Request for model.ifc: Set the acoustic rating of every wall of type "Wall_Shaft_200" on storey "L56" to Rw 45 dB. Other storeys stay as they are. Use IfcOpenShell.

First a look at what the model holds.

```python
import ifcopenshell
import ifcopenshell.util.element

model = ifcopenshell.open("model.ifc")
print(model.schema)
storey = next(s for s in model.by_type("IfcBuildingStorey") if s.Name == "L56")
walls = [e for e in ifcopenshell.util.element.get_decomposition(storey) if e.is_a("IfcWall")]
seen = {}
for e in walls:
    element_type = ifcopenshell.util.element.get_type(e)
    key = (element_type.Name if element_type != e and element_type else None, ifcopenshell.util.element.get_pset(e, "Pset_WallCommon", "AcousticRating"))
    seen[key] = seen.get(key, 0) + 1
for (name, value), count in sorted(seen.items(), key=str):
    print(count, "x", name, "|", value)
```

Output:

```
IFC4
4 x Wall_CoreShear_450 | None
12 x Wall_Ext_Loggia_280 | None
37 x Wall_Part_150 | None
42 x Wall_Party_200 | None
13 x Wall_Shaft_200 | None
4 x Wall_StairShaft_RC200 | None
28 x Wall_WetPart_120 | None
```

```python
import ifcopenshell
import ifcopenshell.api.pset
import ifcopenshell.util.element

model = ifcopenshell.open("model.ifc")

storey = next(s for s in model.by_type("IfcBuildingStorey") if s.Name == "L56")
walls = [e for e in ifcopenshell.util.element.get_decomposition(storey) if e.is_a("IfcWall")]

count = 0
for e in walls:
    element_type = ifcopenshell.util.element.get_type(e)
    if element_type in (None, e) or element_type.Name != "Wall_Shaft_200":
        continue
    found = ifcopenshell.util.element.get_pset(e, "Pset_WallCommon", should_inherit=False)
    if found:
        pset = model.by_id(found["id"])
        if len(ifcopenshell.util.element.get_elements_by_pset(pset)) > 1:
            pset = ifcopenshell.api.pset.unshare_pset(model, products=[e], pset=pset)[0]
    else:
        pset = ifcopenshell.api.pset.add_pset(model, product=e, name="Pset_WallCommon")
    ifcopenshell.api.pset.edit_pset(model, pset=pset, properties={"AcousticRating": "Rw 45 dB"})
    count += 1

print(count, "walls updated")

model.write("model_edited.ifc")
```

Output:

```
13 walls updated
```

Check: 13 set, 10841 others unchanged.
